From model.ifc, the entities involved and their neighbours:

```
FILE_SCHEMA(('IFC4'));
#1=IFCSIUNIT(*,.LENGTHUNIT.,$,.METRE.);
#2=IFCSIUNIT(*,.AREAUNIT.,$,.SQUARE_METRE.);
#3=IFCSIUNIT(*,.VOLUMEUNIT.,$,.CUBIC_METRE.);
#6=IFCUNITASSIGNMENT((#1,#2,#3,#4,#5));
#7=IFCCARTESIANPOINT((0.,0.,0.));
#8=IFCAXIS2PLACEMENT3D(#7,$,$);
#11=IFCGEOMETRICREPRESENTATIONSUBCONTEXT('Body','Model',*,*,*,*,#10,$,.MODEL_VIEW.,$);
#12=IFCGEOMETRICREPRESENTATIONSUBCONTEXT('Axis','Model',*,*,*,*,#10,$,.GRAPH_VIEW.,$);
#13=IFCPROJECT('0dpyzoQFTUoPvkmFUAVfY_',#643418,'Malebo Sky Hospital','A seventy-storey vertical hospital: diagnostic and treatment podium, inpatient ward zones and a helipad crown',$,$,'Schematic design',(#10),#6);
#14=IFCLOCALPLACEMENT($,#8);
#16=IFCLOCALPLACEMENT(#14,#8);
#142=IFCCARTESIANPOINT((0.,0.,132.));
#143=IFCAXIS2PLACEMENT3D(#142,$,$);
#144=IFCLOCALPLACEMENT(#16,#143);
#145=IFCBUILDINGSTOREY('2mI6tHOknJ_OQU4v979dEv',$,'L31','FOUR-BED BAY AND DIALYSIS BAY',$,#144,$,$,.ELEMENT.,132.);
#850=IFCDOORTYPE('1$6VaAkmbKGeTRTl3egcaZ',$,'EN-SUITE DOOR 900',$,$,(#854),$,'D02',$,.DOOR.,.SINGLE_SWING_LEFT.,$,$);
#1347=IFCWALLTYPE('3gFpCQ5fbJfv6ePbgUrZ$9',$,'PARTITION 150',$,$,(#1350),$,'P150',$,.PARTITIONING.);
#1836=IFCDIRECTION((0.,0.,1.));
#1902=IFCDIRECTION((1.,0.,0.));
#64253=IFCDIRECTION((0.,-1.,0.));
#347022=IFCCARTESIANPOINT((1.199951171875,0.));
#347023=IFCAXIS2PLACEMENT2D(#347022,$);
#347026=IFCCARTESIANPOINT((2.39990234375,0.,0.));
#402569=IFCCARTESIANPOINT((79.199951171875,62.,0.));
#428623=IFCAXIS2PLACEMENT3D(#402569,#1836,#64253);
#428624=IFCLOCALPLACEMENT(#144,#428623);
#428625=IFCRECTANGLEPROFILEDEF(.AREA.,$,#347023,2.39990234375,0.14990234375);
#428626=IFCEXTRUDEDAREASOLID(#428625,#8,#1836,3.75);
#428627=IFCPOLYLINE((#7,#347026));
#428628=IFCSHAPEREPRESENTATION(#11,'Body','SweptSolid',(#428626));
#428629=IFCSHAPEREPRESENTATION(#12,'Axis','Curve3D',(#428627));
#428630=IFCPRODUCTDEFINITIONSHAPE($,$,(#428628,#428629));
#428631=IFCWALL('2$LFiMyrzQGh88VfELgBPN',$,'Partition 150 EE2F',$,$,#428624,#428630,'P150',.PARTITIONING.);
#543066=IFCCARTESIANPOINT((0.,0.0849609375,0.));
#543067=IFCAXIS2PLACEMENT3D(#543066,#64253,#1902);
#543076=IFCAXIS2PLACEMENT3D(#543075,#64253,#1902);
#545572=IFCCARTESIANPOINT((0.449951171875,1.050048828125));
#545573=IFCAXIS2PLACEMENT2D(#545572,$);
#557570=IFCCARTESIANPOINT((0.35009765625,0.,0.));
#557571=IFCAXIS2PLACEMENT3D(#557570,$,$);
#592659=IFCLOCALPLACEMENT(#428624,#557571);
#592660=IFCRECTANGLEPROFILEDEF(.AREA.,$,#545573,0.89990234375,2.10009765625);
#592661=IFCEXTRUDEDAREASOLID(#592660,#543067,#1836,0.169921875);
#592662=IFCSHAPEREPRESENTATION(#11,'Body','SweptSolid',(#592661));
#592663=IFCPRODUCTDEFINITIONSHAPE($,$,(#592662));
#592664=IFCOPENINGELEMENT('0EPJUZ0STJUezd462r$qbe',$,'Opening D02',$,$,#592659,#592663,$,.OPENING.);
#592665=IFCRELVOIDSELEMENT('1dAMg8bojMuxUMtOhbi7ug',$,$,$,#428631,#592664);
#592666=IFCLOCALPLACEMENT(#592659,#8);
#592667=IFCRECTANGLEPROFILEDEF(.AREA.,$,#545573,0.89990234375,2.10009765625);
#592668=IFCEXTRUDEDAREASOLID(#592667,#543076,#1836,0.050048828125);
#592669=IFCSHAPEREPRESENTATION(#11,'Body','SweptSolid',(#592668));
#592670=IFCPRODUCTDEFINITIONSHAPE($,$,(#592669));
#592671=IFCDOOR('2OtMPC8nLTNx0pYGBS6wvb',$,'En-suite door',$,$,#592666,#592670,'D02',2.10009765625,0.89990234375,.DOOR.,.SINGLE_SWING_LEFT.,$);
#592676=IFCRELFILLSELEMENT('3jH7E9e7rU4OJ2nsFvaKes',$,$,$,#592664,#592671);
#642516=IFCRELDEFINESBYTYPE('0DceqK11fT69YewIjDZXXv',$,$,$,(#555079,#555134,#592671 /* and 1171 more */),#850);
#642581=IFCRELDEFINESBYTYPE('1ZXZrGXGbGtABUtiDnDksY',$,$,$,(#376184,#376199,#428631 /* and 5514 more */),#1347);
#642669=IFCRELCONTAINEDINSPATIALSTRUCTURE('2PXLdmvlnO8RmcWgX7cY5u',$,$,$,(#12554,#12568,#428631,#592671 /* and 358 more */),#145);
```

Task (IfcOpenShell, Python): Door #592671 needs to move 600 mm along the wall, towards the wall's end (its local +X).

```python
import ifcopenshell
import ifcopenshell.api.geometry
import ifcopenshell.util.placement

model = ifcopenshell.open("model.ifc")

door = model.by_guid("2OtMPC8nLTNx0pYGBS6wvb")
opening = door.FillsVoids[0].RelatingOpeningElement
wall = opening.VoidsElements[0].RelatingBuildingElement

wall_matrix = ifcopenshell.util.placement.get_local_placement(wall.ObjectPlacement)
shift = wall_matrix[:3, 0] * 0.6
before = ifcopenshell.util.placement.get_local_placement(door.ObjectPlacement)[:3, 3].copy()

# The door is placed relative to its opening, so it follows when the opening moves.
matrix = ifcopenshell.util.placement.get_local_placement(opening.ObjectPlacement)
matrix[:3, 3] += shift
ifcopenshell.api.geometry.edit_object_placement(
    model, product=opening, matrix=matrix, is_si=False, should_transform_children=True
)

after = ifcopenshell.util.placement.get_local_placement(door.ObjectPlacement)[:3, 3]
print("door moved by", (after - before).round(3) + 0.0)

model.write("model_rev.ifc")
```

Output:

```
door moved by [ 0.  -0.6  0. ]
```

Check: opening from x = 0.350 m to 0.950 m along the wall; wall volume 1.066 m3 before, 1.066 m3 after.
